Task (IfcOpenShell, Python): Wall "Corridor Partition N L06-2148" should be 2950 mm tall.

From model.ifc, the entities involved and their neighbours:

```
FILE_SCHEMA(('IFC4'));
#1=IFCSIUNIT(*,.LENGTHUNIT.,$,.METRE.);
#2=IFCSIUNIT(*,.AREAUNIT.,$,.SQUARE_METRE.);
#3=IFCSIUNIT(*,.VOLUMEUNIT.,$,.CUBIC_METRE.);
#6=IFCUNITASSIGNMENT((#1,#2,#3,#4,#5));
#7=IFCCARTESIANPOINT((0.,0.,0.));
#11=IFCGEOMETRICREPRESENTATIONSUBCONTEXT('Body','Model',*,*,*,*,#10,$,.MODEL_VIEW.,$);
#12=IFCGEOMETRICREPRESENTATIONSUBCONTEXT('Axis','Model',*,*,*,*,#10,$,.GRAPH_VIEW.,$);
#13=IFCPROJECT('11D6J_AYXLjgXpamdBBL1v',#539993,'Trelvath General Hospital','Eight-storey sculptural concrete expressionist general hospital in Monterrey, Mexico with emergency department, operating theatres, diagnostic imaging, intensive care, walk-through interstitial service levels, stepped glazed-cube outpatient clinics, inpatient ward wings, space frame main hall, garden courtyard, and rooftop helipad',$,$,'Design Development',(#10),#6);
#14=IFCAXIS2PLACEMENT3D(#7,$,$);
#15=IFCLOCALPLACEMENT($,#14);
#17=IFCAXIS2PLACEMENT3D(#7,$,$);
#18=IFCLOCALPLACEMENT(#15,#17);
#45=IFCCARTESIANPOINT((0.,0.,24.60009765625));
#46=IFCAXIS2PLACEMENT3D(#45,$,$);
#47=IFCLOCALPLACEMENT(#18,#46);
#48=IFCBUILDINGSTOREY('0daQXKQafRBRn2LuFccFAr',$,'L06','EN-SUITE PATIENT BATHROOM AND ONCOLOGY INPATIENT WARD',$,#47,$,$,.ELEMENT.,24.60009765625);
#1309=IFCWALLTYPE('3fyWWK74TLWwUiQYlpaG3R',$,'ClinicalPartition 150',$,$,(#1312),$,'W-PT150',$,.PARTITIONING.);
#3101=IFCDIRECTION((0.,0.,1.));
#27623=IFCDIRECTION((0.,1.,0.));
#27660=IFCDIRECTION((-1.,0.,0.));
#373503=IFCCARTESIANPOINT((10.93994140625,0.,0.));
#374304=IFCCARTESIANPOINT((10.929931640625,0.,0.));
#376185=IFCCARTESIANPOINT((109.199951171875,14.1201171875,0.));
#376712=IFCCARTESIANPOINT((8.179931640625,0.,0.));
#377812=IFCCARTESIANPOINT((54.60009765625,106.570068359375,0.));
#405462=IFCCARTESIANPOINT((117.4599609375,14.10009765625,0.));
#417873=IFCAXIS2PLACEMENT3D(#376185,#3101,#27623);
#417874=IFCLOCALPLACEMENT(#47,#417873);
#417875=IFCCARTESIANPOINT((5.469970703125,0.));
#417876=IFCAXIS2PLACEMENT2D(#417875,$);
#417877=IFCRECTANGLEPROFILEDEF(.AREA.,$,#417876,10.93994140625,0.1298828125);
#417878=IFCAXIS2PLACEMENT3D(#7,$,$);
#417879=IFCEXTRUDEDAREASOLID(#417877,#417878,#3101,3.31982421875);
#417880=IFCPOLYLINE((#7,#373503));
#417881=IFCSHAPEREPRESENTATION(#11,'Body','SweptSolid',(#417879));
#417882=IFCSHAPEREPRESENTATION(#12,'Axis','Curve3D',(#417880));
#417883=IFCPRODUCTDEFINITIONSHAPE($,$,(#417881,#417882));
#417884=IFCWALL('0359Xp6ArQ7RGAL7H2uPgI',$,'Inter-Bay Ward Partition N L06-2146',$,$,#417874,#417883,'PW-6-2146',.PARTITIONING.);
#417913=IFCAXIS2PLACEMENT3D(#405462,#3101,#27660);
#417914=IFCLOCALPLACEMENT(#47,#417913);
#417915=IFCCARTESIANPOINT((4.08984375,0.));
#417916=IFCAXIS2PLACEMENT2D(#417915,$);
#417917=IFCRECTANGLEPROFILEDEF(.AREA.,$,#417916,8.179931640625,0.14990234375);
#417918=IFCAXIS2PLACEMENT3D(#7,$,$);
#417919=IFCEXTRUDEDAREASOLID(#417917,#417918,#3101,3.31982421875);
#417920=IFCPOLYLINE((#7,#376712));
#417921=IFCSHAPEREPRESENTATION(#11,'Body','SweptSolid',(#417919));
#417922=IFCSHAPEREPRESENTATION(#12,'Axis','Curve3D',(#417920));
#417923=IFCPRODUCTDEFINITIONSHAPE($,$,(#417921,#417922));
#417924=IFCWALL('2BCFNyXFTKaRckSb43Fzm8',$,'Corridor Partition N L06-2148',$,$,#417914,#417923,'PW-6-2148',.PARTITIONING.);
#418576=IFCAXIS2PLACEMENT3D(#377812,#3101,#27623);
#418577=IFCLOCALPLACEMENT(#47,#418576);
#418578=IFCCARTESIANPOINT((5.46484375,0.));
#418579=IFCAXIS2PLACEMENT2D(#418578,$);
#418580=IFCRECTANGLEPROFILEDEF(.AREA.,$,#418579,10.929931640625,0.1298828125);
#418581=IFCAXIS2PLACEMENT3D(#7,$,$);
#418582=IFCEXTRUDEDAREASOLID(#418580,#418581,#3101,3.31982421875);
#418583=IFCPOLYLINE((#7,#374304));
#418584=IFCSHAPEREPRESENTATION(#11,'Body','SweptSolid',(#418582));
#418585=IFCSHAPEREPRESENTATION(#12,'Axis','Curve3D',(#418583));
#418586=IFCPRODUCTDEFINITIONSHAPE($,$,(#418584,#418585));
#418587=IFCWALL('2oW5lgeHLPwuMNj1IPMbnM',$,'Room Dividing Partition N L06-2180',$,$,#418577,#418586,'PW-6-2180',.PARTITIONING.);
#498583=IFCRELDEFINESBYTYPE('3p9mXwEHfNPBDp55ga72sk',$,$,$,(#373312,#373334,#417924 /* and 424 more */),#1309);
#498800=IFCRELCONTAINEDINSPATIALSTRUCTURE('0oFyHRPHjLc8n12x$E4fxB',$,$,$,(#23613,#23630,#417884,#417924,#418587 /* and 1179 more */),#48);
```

```python
import ifcopenshell
import ifcopenshell.geom
import ifcopenshell.util.representation
import ifcopenshell.util.shape

model = ifcopenshell.open("model.ifc")
settings = ifcopenshell.geom.settings()


def volume(element):
    """Net volume in cubic metres, openings subtracted."""
    shape = ifcopenshell.geom.create_shape(settings, element)
    return ifcopenshell.util.shape.get_volume(shape.geometry)


wall = model.by_guid("2BCFNyXFTKaRckSb43Fzm8")
before = volume(wall)

body = ifcopenshell.util.representation.get_representation(wall, "Model", "Body")
solid = body.Items[0]
old_height = solid.Depth
solid.Depth = 2.95
after = volume(wall)

print(f"height {old_height:g} -> {solid.Depth:g}, volume {before:.3f} -> {after:.3f} m3")

model.write("model_v2.ifc")
```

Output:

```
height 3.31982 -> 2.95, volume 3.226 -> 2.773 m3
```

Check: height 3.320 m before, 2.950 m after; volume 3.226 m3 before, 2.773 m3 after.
